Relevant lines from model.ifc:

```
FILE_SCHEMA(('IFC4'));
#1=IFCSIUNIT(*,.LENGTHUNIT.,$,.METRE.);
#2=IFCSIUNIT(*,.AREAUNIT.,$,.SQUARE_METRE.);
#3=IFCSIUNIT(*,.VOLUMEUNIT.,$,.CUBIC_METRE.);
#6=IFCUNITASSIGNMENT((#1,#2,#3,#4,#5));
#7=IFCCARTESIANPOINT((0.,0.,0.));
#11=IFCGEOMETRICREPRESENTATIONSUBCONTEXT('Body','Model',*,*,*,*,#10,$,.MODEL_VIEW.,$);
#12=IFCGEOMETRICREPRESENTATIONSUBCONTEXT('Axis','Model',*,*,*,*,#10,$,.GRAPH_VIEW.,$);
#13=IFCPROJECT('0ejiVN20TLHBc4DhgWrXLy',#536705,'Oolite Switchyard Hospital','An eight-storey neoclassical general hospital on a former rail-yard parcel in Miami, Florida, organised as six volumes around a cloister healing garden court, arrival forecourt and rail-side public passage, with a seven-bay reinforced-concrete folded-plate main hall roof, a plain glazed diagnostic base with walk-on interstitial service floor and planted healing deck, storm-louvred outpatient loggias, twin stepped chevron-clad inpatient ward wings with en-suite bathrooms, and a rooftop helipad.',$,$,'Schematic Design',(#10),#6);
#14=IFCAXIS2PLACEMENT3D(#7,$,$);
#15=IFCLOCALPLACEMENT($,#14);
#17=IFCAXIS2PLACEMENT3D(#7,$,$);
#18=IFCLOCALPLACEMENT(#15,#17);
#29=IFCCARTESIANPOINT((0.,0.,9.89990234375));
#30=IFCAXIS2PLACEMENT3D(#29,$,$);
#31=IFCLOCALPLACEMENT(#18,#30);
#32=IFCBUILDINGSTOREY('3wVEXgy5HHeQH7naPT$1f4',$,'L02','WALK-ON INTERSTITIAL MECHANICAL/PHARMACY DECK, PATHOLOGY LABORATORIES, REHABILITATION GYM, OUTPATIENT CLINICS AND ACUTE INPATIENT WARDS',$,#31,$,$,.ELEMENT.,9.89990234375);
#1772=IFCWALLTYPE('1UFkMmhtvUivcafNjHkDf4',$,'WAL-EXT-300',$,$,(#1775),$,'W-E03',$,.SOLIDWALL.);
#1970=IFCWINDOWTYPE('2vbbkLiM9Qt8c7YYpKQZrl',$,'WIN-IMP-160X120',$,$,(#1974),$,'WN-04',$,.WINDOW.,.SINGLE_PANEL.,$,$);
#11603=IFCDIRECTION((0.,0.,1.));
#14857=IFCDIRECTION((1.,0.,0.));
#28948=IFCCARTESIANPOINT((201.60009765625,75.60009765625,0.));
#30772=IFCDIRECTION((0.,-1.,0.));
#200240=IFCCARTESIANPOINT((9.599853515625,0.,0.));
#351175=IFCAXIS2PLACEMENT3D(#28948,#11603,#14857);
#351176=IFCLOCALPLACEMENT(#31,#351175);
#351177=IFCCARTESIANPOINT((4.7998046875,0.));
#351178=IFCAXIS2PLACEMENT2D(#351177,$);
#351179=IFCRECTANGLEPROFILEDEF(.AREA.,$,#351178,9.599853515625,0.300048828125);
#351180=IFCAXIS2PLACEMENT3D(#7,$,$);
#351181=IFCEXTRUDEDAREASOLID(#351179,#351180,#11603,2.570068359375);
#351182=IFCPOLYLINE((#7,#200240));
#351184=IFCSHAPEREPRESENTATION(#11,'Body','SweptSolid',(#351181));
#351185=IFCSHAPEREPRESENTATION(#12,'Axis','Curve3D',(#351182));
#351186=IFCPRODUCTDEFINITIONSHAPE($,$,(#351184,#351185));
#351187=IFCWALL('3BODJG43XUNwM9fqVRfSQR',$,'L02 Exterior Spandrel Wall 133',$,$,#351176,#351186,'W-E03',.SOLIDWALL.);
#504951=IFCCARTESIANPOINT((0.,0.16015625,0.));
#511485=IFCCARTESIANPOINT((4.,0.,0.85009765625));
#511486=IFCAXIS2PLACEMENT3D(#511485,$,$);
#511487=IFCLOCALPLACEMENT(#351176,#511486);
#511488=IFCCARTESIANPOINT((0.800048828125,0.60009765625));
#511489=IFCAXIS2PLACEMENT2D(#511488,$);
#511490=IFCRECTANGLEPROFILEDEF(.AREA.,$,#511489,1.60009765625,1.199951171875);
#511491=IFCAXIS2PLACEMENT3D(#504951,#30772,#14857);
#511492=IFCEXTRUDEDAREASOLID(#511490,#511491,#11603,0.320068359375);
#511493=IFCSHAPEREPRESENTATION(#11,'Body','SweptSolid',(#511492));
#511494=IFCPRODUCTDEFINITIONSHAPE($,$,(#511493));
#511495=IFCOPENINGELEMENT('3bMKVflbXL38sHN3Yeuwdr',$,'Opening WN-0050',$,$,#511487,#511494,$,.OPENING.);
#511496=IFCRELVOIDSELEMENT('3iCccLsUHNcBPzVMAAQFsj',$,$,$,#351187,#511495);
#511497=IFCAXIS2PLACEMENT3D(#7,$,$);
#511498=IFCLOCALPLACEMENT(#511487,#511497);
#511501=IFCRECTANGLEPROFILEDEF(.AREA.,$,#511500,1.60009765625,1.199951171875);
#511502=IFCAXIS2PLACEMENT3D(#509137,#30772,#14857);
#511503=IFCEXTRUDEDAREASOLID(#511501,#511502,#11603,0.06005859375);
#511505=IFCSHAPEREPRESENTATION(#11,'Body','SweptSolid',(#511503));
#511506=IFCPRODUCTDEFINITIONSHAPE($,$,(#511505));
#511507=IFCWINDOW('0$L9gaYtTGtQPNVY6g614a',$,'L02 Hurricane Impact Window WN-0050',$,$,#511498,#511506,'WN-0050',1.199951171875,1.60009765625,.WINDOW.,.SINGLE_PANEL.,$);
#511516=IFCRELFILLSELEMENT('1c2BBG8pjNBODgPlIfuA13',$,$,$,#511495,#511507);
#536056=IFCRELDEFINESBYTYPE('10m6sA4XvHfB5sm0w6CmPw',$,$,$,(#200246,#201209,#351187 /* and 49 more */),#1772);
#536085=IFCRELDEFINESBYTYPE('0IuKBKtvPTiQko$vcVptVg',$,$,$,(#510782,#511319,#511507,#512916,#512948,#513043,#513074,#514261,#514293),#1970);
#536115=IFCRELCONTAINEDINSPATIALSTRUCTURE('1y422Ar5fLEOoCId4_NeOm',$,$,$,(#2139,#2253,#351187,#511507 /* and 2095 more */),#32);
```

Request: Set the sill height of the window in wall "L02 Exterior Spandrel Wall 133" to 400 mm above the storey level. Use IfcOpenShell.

```python
import numpy as np
import ifcopenshell
import ifcopenshell.api.geometry
import ifcopenshell.geom
import ifcopenshell.util.element
import ifcopenshell.util.placement
import ifcopenshell.util.shape
import ifcopenshell.util.unit

model = ifcopenshell.open("model.ifc")
unit_scale = ifcopenshell.util.unit.calculate_unit_scale(model)

window = model.by_guid("0$L9gaYtTGtQPNVY6g614a")
opening = window.FillsVoids[0].RelatingOpeningElement
storey = ifcopenshell.util.element.get_container(window, ifc_class="IfcBuildingStorey")
level = ifcopenshell.util.placement.get_local_placement(storey.ObjectPlacement)[2, 3]

# The opening's origin need not be at the sill, so measure its lowest point.
shape = ifcopenshell.geom.create_shape(ifcopenshell.geom.settings(), opening)
bottom = ifcopenshell.util.shape.get_shape_bottom_elevation(shape, shape.geometry) / unit_scale
dz = level + 0.4 / unit_scale - bottom

shift = np.array([0.0, 0.0, dz])
# The window is placed relative to its opening, so it follows when the opening moves.
matrix = ifcopenshell.util.placement.get_local_placement(opening.ObjectPlacement)
matrix[:3, 3] += shift
ifcopenshell.api.geometry.edit_object_placement(
    model, product=opening, matrix=matrix, is_si=False, should_transform_children=True
)

print(f"moved by {dz * unit_scale:+.3f} m")

model.write("model-out.ifc")
```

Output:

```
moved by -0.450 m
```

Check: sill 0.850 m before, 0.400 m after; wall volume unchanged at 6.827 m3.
